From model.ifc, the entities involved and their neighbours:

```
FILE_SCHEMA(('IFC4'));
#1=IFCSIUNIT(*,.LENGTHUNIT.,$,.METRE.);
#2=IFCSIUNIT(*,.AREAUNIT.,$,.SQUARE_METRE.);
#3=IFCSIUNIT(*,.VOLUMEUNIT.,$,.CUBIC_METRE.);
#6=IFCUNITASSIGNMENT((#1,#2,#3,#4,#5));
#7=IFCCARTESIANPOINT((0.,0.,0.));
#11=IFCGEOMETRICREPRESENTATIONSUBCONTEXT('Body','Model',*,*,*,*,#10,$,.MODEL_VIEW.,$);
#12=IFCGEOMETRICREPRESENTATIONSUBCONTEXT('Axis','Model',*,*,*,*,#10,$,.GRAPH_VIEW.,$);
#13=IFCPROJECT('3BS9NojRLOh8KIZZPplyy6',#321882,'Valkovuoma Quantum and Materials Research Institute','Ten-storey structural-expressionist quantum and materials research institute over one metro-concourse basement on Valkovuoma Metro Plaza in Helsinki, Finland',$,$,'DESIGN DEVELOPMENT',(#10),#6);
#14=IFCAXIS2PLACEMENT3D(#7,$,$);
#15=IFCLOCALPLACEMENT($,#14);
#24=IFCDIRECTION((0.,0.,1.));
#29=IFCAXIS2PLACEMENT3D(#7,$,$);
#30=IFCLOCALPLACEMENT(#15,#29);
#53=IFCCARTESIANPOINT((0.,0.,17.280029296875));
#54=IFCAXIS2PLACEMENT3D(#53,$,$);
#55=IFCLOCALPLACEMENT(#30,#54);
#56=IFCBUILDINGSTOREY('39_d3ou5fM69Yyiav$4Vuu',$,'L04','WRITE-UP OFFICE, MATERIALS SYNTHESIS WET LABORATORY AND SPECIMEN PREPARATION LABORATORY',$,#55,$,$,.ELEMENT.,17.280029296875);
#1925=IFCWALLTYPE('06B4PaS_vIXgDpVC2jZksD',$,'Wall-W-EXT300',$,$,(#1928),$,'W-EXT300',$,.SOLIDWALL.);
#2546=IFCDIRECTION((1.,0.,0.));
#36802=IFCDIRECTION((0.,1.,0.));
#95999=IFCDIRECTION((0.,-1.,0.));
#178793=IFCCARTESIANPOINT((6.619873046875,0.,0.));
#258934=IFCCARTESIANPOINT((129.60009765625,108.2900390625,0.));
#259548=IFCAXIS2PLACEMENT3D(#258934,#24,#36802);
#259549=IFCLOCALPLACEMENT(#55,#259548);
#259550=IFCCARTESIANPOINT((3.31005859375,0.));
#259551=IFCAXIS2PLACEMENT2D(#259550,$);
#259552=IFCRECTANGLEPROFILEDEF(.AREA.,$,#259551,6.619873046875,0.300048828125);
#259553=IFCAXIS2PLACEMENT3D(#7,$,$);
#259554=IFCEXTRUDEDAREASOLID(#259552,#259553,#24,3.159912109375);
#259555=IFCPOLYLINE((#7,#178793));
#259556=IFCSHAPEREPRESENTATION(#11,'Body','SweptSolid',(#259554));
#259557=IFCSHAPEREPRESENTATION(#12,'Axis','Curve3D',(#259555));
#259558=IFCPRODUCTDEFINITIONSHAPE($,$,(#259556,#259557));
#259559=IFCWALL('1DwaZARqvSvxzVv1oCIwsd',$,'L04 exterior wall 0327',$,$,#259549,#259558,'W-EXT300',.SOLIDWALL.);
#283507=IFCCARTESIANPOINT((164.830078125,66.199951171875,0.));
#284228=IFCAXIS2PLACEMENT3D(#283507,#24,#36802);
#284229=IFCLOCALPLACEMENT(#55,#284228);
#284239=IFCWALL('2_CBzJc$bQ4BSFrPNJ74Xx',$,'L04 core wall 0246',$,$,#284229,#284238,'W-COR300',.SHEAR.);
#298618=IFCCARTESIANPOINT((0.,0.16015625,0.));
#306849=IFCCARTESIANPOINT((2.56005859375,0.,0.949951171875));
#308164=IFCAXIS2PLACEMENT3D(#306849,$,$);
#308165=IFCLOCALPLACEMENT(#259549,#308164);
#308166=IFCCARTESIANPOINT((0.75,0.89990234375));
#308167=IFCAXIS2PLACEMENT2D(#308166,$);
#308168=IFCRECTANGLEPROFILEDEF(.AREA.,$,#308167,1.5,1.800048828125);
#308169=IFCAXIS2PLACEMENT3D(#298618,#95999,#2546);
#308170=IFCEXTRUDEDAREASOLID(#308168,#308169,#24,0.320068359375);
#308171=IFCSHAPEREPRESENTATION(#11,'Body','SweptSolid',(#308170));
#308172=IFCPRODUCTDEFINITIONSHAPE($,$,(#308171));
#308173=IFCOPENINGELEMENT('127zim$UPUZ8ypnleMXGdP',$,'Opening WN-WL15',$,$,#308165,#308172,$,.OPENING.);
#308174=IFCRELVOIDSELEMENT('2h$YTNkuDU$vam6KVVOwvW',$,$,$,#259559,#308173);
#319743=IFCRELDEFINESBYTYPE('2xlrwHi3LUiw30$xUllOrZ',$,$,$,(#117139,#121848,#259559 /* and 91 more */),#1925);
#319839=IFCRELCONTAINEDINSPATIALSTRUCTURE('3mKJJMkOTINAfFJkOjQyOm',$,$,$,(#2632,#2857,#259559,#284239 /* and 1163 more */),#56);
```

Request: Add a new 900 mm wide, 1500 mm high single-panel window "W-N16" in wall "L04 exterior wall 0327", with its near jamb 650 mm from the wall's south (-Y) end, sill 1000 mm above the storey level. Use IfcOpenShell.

```python
import numpy as np
import ifcopenshell
import ifcopenshell.api.feature
import ifcopenshell.api.geometry
import ifcopenshell.api.root
import ifcopenshell.api.spatial
import ifcopenshell.geom
import ifcopenshell.util.element
import ifcopenshell.util.placement
import ifcopenshell.util.representation
import ifcopenshell.util.shape
import ifcopenshell.util.unit

model = ifcopenshell.open("model.ifc")
unit_scale = ifcopenshell.util.unit.calculate_unit_scale(model)
settings = ifcopenshell.geom.settings()


def volume(element):
    """Net volume in cubic metres, openings subtracted."""
    shape = ifcopenshell.geom.create_shape(settings, element)
    return ifcopenshell.util.shape.get_volume(shape.geometry)


wall = model.by_guid("1DwaZARqvSvxzVv1oCIwsd")
storey = ifcopenshell.util.element.get_container(wall, ifc_class="IfcBuildingStorey")
context = ifcopenshell.util.representation.get_context(model, "Model", "Body", "MODEL_VIEW")
before = volume(wall)

width, height, from_end, sill = 0.9, 1.5, 0.65, 1  # metres

# The wall runs along its own X axis, and the end named is its -X end.
wall_shape = ifcopenshell.geom.create_shape(settings, wall)
x, y, z = ifcopenshell.util.shape.get_vertices(wall_shape.geometry).T
start = x.min() + from_end
face, thickness = float(y.min()), float(y.max() - y.min())
wall_matrix = ifcopenshell.util.placement.get_local_placement(wall.ObjectPlacement)
level = ifcopenshell.util.placement.get_local_placement(storey.ObjectPlacement)[2, 3]


def in_wall(x, y):
    """Placement at x, y metres in the wall's axes, at sill height."""
    matrix = wall_matrix.copy()
    matrix[:, 3] = wall_matrix @ np.array([x / unit_scale, y / unit_scale, 0.0, 1.0])
    matrix[2, 3] = level + sill / unit_scale
    return matrix


# Opening: a box that overshoots both wall faces by 50 mm.
opening = ifcopenshell.api.root.create_entity(model, ifc_class="IfcOpeningElement", predefined_type="OPENING")
box = ifcopenshell.api.geometry.add_wall_representation(
    model, context=context, length=width, height=height, thickness=thickness + 0.1
)
ifcopenshell.api.geometry.assign_representation(model, product=opening, representation=box)
ifcopenshell.api.geometry.edit_object_placement(model, product=opening, matrix=in_wall(start, face - 0.05), is_si=False)
ifcopenshell.api.feature.add_feature(model, feature=opening, element=wall)

window = ifcopenshell.api.root.create_entity(model, ifc_class="IfcWindow", name="W-N16", predefined_type="WINDOW")
window.OverallWidth, window.OverallHeight = width / unit_scale, height / unit_scale
window.PartitioningType = "SINGLE_PANEL"
body = ifcopenshell.api.geometry.add_window_representation(
    model,
    context=context,
    overall_width=window.OverallWidth,
    overall_height=window.OverallHeight,
    partition_type="SINGLE_PANEL",
)
ifcopenshell.api.geometry.assign_representation(model, product=window, representation=body)
ifcopenshell.api.spatial.assign_container(model, products=[window], relating_structure=storey)
ifcopenshell.api.feature.add_filling(model, opening=opening, element=window)

# Centre the window in the wall's thickness.
ifcopenshell.api.geometry.edit_object_placement(model, product=window, matrix=in_wall(start, face), is_si=False)
window_shape = ifcopenshell.geom.create_shape(settings, window)
depth = ifcopenshell.util.shape.get_vertices(window_shape.geometry)[:, 1]
offset = face + thickness / 2 - (depth.min() + depth.max()) / 2
ifcopenshell.api.geometry.edit_object_placement(model, product=window, matrix=in_wall(start, offset), is_si=False)

after = volume(wall)

print(f"wall volume {before:.3f} -> {after:.3f} m3")

model.write("model_rev.ifc")
```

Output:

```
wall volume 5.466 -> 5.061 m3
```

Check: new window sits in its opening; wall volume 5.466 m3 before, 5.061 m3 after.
